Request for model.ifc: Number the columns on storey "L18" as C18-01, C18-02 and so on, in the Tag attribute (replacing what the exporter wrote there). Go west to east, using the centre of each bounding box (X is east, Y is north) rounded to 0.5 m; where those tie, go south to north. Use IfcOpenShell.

First a look at what the model holds.

```python
import ifcopenshell
import ifcopenshell.util.element
import ifcopenshell.util.placement

model = ifcopenshell.open("model.ifc")
print(model.schema)
storey = next(s for s in model.by_type("IfcBuildingStorey") if s.Name == "L18")
columns = [e for e in ifcopenshell.util.element.get_decomposition(storey) if e.is_a("IfcColumn")]
for e in sorted(columns, key=lambda e: e.id()):
    origin = ifcopenshell.util.placement.get_local_placement(e.ObjectPlacement)[:3, 3]
    print(e.id(), e.Tag, e.Name, origin.round(2) + 0.0, sep=" | ")
```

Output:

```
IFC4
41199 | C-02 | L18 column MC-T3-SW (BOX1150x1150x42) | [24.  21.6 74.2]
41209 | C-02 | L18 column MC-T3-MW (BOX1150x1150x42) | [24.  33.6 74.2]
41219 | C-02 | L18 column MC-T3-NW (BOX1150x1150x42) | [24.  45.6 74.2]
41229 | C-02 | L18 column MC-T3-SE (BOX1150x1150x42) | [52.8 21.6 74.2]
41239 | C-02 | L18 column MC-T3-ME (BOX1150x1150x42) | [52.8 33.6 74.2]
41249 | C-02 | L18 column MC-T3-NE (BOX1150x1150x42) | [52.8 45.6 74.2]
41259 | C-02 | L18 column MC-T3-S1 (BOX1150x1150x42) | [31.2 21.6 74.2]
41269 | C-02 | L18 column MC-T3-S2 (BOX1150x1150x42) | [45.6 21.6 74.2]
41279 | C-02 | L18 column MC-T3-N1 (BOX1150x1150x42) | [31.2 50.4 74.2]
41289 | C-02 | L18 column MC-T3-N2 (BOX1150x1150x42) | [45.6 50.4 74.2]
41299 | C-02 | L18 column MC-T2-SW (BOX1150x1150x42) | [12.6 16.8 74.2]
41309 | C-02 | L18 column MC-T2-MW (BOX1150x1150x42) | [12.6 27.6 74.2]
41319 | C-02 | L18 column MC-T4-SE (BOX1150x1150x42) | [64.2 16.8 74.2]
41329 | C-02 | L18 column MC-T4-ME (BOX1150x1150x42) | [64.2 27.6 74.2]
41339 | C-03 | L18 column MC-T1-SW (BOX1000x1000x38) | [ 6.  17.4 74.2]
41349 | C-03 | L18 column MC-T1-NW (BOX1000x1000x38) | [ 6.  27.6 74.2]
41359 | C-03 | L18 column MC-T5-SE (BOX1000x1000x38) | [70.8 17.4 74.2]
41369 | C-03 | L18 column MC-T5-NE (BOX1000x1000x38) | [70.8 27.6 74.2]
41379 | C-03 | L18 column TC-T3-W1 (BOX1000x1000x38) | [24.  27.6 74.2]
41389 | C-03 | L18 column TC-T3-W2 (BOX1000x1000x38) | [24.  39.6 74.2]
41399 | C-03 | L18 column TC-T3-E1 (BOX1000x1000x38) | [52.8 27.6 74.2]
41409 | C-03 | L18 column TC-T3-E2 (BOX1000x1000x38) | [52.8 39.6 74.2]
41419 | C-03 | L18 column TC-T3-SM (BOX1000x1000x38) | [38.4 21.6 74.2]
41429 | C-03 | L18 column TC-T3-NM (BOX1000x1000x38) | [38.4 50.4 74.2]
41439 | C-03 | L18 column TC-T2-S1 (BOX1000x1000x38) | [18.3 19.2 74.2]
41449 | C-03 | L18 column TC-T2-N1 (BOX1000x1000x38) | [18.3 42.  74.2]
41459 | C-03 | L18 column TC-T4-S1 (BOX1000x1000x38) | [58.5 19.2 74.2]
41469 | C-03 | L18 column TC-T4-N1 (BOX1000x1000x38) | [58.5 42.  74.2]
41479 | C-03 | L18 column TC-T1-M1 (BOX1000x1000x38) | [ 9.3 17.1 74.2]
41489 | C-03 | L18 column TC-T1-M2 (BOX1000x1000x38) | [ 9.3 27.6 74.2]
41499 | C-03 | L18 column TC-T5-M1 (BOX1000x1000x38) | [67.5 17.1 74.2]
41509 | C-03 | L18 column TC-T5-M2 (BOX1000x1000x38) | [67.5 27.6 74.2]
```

```python
import ifcopenshell
import ifcopenshell.geom
import ifcopenshell.util.element
import ifcopenshell.util.shape

model = ifcopenshell.open("model.ifc")
settings = ifcopenshell.geom.settings()
settings.set("use-world-coords", True)


def centre(element):
    shape = ifcopenshell.geom.create_shape(settings, element)
    return ifcopenshell.util.shape.get_bbox_centroid(shape.geometry)


storey = next(s for s in model.by_type("IfcBuildingStorey") if s.Name == "L18")
columns = [e for e in ifcopenshell.util.element.get_decomposition(storey) if e.is_a("IfcColumn")]

# Insertion points can sit at a corner or the storey origin, so sort by the geometry (in metres).
centres = {e: centre(e) for e in columns}
columns.sort(key=lambda e: (round(centres[e][0] / 0.5), centres[e][1]))

for i, e in enumerate(columns, start=1):
    number = f"C18-{i:02d}"
    e.Tag = number
    print(e.id(), number)

model.write("model-out.ifc")
```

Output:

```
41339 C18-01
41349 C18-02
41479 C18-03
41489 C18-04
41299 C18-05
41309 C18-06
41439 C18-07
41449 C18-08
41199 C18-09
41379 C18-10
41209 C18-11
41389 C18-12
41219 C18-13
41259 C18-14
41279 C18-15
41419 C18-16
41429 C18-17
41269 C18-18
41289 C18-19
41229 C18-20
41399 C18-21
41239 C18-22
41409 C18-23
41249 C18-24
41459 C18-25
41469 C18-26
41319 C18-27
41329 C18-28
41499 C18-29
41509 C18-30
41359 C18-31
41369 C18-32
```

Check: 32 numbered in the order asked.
